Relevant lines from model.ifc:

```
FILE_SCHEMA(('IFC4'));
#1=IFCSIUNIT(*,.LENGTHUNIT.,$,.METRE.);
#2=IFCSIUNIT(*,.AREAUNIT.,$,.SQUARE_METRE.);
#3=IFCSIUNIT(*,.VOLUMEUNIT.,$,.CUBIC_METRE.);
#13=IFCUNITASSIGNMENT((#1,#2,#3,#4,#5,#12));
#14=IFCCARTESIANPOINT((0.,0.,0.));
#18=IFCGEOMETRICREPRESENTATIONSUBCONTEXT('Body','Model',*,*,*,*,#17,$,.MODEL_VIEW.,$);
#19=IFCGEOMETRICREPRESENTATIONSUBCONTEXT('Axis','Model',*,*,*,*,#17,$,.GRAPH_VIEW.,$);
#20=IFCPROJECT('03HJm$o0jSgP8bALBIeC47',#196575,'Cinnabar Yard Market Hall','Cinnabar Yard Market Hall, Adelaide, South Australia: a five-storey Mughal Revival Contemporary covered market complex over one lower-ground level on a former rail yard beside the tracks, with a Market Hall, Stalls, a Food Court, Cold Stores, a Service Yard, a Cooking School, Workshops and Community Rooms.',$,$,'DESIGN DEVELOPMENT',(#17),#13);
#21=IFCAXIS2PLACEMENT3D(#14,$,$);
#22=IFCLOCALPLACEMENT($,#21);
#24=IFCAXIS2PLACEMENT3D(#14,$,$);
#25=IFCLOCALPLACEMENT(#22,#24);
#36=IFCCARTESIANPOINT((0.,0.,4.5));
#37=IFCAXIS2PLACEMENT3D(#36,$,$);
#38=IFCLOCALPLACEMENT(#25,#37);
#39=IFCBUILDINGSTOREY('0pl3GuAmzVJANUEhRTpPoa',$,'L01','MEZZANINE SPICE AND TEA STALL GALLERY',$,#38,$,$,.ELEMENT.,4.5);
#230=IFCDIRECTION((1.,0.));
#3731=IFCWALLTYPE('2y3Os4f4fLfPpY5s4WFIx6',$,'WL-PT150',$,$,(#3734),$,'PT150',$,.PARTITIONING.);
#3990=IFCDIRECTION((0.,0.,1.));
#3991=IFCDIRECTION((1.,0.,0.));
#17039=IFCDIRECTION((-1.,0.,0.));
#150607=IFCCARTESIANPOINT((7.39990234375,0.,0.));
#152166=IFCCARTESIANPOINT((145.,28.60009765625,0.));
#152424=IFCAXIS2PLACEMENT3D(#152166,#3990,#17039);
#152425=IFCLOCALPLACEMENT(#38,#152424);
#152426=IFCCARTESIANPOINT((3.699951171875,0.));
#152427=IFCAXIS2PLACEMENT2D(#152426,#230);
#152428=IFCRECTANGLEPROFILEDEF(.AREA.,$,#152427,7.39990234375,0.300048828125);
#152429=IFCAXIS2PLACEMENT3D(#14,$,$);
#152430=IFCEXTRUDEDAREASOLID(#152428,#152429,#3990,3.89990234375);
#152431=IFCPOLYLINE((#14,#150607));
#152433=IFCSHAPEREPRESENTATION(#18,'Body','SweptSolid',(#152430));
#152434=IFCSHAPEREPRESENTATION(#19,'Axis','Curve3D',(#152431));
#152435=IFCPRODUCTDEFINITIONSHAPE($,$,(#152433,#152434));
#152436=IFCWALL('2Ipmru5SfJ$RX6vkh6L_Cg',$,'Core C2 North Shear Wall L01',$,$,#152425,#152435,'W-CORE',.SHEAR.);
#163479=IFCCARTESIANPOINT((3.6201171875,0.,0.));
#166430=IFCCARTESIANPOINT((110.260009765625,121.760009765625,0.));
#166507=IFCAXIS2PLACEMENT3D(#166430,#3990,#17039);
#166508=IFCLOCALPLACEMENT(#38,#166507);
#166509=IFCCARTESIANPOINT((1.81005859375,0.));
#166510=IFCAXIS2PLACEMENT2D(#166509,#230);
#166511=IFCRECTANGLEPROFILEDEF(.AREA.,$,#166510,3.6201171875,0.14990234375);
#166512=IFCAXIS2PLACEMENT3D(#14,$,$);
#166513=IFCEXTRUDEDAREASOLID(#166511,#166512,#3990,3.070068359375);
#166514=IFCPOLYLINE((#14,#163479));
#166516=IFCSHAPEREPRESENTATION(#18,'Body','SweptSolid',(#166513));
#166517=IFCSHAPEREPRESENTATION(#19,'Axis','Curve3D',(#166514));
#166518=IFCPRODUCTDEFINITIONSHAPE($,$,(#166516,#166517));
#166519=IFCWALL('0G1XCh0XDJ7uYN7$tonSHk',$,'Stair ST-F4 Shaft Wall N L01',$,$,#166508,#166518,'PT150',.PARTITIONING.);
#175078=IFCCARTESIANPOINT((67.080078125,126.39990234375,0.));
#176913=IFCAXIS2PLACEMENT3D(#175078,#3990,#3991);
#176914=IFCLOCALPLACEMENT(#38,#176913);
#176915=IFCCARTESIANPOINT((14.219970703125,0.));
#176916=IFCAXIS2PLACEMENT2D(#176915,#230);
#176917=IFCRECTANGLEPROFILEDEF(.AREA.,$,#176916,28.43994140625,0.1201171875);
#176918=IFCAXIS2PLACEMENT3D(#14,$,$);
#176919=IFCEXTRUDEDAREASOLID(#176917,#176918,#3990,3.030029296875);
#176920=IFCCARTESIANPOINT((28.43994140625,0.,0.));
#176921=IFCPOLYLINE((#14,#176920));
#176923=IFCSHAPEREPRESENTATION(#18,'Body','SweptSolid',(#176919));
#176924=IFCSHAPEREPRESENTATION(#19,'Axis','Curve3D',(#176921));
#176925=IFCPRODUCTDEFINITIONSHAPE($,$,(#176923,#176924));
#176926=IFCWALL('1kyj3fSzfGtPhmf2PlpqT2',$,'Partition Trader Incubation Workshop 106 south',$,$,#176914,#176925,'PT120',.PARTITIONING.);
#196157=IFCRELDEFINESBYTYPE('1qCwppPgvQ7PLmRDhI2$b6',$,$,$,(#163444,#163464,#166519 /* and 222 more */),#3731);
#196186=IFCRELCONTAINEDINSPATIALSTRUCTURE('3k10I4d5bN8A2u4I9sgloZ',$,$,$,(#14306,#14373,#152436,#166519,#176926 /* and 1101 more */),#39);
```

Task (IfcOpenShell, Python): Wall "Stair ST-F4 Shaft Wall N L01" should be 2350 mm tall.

```python
import ifcopenshell
import ifcopenshell.geom
import ifcopenshell.util.representation
import ifcopenshell.util.shape
import ifcopenshell.util.unit

model = ifcopenshell.open("model.ifc")
unit_scale = ifcopenshell.util.unit.calculate_unit_scale(model)
settings = ifcopenshell.geom.settings()


def volume(element):
    """Net volume in cubic metres, openings subtracted."""
    shape = ifcopenshell.geom.create_shape(settings, element)
    return ifcopenshell.util.shape.get_volume(shape.geometry)


wall = model.by_id(166519)
before = volume(wall)

body = ifcopenshell.util.representation.get_representation(wall, "Model", "Body")
solid = body.Items[0]
old_height = solid.Depth
solid.Depth = 2.35 / unit_scale
after = volume(wall)

print(f"height {old_height:g} -> {solid.Depth:g}, volume {before:.3f} -> {after:.3f} m3")

model.write("model-out.ifc")
```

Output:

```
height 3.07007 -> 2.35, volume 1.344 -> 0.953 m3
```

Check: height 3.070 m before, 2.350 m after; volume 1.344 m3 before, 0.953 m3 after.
